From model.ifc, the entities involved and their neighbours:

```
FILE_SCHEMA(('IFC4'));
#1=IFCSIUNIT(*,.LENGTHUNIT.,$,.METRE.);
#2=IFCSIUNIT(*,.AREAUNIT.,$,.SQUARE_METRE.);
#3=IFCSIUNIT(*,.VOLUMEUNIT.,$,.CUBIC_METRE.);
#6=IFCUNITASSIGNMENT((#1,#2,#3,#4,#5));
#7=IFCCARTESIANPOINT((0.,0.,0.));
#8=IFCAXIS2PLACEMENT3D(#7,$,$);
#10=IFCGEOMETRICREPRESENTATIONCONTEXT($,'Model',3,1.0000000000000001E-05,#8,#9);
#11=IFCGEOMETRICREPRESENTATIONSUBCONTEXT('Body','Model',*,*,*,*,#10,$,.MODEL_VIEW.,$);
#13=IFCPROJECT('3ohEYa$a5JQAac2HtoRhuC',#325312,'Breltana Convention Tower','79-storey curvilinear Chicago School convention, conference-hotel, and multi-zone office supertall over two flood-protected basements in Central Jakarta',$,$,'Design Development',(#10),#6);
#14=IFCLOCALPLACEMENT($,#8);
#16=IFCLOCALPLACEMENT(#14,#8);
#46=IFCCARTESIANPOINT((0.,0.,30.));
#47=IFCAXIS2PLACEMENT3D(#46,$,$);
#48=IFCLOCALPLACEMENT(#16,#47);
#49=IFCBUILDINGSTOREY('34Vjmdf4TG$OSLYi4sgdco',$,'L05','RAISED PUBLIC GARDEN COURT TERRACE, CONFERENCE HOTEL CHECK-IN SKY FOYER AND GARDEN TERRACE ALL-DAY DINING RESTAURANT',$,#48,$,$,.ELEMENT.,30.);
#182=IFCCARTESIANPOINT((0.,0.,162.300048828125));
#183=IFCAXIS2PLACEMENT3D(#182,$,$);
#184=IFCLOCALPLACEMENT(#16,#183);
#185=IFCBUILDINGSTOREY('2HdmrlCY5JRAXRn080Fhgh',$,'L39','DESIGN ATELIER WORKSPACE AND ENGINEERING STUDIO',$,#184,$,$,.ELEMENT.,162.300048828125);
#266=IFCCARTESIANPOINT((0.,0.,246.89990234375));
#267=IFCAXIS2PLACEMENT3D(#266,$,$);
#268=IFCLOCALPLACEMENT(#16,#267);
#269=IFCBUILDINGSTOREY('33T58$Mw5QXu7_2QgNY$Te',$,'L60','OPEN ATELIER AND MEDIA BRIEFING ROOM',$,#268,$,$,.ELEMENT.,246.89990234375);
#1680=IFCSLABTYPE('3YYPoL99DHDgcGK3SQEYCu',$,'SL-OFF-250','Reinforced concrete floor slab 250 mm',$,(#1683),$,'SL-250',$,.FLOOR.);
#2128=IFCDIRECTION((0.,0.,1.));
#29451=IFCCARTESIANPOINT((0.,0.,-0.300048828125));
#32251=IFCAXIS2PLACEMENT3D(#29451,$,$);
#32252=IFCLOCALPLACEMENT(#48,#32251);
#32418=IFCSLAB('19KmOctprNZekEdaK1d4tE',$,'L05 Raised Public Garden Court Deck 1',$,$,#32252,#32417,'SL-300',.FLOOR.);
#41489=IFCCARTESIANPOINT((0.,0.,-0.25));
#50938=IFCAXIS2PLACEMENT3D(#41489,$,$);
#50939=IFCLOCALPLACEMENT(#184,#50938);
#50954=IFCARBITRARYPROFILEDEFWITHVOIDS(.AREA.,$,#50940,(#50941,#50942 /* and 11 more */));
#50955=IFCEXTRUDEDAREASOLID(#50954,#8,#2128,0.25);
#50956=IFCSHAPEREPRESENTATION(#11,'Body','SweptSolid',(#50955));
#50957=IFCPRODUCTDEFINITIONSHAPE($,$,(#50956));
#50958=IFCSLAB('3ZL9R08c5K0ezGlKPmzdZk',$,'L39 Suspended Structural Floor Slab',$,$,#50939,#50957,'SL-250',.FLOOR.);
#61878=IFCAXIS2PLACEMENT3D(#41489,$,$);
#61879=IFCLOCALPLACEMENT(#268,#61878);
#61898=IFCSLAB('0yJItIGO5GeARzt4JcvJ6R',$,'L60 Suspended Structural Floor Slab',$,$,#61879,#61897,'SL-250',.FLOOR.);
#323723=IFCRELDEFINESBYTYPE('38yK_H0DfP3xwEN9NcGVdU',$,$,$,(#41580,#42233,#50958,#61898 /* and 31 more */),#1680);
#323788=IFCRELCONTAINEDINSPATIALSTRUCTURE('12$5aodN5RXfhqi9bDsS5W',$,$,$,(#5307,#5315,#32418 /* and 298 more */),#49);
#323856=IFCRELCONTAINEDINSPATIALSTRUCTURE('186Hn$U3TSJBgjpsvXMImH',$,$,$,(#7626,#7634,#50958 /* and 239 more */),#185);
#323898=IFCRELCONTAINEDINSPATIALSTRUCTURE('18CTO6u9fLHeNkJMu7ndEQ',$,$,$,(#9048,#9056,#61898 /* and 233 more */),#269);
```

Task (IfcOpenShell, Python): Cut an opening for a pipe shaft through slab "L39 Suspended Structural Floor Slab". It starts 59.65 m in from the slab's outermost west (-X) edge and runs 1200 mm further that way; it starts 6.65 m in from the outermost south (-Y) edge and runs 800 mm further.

```python
import numpy as np
import ifcopenshell
import ifcopenshell.api.feature
import ifcopenshell.api.geometry
import ifcopenshell.api.root
import ifcopenshell.geom
import ifcopenshell.util.placement
import ifcopenshell.util.representation
import ifcopenshell.util.shape
import ifcopenshell.util.unit

model = ifcopenshell.open("model.ifc")
unit_scale = ifcopenshell.util.unit.calculate_unit_scale(model)
settings = ifcopenshell.geom.settings()


def volume(element):
    """Net volume in cubic metres, openings subtracted."""
    shape = ifcopenshell.geom.create_shape(settings, element)
    return ifcopenshell.util.shape.get_volume(shape.geometry)


slab = model.by_guid("3ZL9R08c5K0ezGlKPmzdZk")
before = volume(slab)

# Extent in the slab's own axes, in metres. The edges named are its -X and -Y sides.
slab_shape = ifcopenshell.geom.create_shape(settings, slab)
vertices = ifcopenshell.util.shape.get_vertices(slab_shape.geometry)
x_min, y_min, bottom = vertices.min(axis=0)
top = vertices[:, 2].max()

opening = ifcopenshell.api.root.create_entity(model, ifc_class="IfcOpeningElement", name="Pipe shaft opening", predefined_type="OPENING")
context = ifcopenshell.util.representation.get_context(model, "Model", "Body", "MODEL_VIEW")
width, depth = 1.2, 0.8
outline = [(0.0, 0.0), (width, 0.0), (width, depth), (0.0, depth), (0.0, 0.0)]
# Overshoot both faces by 50 mm so the cut is clean.
shape = ifcopenshell.api.geometry.add_slab_representation(
    model, context=context, depth=top - bottom + 0.1, polyline=outline
)
ifcopenshell.api.geometry.assign_representation(model, product=opening, representation=shape)

matrix = ifcopenshell.util.placement.get_local_placement(slab.ObjectPlacement)
matrix[:, 3] = matrix @ np.append(np.array([x_min + 59.65, y_min + 6.65, bottom - 0.05]) / unit_scale, 1.0)
ifcopenshell.api.geometry.edit_object_placement(model, product=opening, matrix=matrix, is_si=False)
ifcopenshell.api.feature.add_feature(model, feature=opening, element=slab)

after = volume(slab)

print(f"slab volume {before:.3f} -> {after:.3f} m3")

model.write("model-out.ifc")
```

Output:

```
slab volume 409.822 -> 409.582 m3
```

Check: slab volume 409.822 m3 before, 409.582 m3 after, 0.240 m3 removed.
